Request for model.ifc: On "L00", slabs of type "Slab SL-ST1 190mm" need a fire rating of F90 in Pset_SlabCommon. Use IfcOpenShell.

First a look at what the model holds.

```python
import ifcopenshell
import ifcopenshell.util.element

model = ifcopenshell.open("model.ifc")
print(model.schema)
storey = next(s for s in model.by_type("IfcBuildingStorey") if s.Name == "L00")
slabs = [e for e in ifcopenshell.util.element.get_decomposition(storey) if e.is_a("IfcSlab")]
seen = {}
for e in slabs:
    element_type = ifcopenshell.util.element.get_type(e)
    key = (element_type.Name if element_type != e and element_type else None, ifcopenshell.util.element.get_pset(e, "Pset_SlabCommon", "FireRating"))
    seen[key] = seen.get(key, 0) + 1
for (name, value), count in sorted(seen.items(), key=str):
    print(count, "x", name, "|", value)
```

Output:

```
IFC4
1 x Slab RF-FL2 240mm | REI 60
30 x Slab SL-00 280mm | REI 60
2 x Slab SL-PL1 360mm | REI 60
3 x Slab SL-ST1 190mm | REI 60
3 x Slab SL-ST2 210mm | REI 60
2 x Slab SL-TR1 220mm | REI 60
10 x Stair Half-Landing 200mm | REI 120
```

```python
import ifcopenshell
import ifcopenshell.api.pset
import ifcopenshell.util.element

model = ifcopenshell.open("model.ifc")

storey = next(s for s in model.by_type("IfcBuildingStorey") if s.Name == "L00")
slabs = [e for e in ifcopenshell.util.element.get_decomposition(storey) if e.is_a("IfcSlab")]

count = 0
for e in slabs:
    element_type = ifcopenshell.util.element.get_type(e)
    if element_type in (None, e) or element_type.Name != "Slab SL-ST1 190mm":
        continue
    # add_pset returns the element's existing set when there is one.
    pset = ifcopenshell.api.pset.add_pset(model, product=e, name="Pset_SlabCommon")
    ifcopenshell.api.pset.edit_pset(model, pset=pset, properties={"FireRating": "F90"})
    count += 1

print(count, "slabs updated")

model.write("model_v2.ifc")
```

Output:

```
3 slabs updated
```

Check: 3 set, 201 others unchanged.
